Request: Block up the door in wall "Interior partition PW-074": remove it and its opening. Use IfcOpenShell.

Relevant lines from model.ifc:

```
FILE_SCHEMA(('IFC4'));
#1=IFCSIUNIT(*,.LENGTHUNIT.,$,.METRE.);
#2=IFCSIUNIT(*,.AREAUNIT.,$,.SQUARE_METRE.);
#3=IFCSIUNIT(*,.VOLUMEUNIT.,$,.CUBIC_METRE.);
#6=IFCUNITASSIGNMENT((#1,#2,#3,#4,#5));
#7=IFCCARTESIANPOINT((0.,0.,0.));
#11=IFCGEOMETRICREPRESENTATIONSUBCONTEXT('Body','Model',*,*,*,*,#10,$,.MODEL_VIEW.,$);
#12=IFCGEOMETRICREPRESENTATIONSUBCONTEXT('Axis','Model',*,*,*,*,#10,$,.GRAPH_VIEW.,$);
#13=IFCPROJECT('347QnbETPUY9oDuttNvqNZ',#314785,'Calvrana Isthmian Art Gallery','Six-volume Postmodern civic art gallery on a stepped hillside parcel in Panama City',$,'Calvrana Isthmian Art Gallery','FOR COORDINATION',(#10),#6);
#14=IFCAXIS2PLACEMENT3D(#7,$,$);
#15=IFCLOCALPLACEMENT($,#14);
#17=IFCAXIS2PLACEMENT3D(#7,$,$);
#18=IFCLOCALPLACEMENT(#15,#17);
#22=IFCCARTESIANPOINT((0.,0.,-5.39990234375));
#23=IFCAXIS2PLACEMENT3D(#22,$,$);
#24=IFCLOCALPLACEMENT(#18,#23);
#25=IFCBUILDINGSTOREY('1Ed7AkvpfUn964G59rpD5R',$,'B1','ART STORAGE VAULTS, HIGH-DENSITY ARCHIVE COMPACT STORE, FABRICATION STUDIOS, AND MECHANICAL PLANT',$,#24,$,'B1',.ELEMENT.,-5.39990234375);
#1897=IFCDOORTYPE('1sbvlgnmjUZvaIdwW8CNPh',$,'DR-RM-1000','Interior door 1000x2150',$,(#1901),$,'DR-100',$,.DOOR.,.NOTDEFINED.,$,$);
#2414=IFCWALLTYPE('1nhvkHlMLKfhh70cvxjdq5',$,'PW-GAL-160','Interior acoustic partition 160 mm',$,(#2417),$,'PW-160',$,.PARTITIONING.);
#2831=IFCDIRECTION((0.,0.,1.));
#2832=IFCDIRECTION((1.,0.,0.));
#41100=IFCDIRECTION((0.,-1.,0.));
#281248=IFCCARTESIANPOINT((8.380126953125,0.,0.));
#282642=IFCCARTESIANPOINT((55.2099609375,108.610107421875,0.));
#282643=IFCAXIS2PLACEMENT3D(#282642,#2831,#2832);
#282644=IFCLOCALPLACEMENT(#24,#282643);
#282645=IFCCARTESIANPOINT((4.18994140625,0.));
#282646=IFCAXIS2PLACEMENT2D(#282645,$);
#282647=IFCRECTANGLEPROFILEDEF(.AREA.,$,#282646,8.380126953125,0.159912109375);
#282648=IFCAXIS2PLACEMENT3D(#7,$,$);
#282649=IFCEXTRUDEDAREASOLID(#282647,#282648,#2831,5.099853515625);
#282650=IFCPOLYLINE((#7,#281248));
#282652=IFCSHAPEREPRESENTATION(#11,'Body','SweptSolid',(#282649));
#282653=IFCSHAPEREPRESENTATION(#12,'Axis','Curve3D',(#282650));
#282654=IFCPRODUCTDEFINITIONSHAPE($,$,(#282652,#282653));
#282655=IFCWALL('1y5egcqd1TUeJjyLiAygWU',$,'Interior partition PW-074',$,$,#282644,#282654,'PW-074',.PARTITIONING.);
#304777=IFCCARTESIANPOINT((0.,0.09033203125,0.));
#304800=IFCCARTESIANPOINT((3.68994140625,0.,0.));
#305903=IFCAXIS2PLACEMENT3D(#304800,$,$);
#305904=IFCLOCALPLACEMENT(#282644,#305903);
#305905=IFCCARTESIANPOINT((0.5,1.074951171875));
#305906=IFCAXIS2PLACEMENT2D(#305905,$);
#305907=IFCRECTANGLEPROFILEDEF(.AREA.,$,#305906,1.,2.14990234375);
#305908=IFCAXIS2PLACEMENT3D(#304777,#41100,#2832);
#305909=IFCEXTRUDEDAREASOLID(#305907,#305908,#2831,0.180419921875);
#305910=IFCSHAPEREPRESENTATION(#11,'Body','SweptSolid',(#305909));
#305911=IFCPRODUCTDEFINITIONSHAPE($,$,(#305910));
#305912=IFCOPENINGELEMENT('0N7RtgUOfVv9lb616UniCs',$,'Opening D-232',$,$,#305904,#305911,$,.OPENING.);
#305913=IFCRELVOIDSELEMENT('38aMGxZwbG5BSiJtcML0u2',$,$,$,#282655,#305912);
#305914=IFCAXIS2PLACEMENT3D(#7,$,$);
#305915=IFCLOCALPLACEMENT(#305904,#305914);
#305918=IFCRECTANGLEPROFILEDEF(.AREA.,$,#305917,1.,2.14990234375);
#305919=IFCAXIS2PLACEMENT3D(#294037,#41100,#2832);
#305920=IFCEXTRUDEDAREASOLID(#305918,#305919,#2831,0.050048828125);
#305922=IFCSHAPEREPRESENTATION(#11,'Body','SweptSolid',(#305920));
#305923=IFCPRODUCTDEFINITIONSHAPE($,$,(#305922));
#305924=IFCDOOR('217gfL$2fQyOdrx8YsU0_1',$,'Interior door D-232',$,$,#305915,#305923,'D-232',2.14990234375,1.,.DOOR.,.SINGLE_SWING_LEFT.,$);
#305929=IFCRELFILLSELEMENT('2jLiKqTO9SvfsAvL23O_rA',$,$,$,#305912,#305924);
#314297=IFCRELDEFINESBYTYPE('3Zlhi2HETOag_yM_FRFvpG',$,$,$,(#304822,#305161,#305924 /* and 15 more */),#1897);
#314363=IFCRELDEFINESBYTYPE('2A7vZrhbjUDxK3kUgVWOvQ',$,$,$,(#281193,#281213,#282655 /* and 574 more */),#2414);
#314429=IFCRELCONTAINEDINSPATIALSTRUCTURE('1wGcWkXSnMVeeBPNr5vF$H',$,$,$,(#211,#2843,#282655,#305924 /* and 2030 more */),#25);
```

```python
import ifcopenshell
import ifcopenshell.api.feature
import ifcopenshell.api.root
import ifcopenshell.geom
import ifcopenshell.util.shape

model = ifcopenshell.open("model.ifc")
settings = ifcopenshell.geom.settings()


def volume(element):
    """Net volume in cubic metres, openings subtracted."""
    shape = ifcopenshell.geom.create_shape(settings, element)
    return ifcopenshell.util.shape.get_volume(shape.geometry)


door = model.by_guid("217gfL$2fQyOdrx8YsU0_1")
opening = door.FillsVoids[0].RelatingOpeningElement
wall = opening.VoidsElements[0].RelatingBuildingElement
before = volume(wall)

ifcopenshell.api.root.remove_product(model, product=door)
ifcopenshell.api.feature.remove_feature(model, feature=opening)

after = volume(wall)

print(f"wall volume {before:.3f} -> {after:.3f} m3")

model.write("model_v2.ifc")
```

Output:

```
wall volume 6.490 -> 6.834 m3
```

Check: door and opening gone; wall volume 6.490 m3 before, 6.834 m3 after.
